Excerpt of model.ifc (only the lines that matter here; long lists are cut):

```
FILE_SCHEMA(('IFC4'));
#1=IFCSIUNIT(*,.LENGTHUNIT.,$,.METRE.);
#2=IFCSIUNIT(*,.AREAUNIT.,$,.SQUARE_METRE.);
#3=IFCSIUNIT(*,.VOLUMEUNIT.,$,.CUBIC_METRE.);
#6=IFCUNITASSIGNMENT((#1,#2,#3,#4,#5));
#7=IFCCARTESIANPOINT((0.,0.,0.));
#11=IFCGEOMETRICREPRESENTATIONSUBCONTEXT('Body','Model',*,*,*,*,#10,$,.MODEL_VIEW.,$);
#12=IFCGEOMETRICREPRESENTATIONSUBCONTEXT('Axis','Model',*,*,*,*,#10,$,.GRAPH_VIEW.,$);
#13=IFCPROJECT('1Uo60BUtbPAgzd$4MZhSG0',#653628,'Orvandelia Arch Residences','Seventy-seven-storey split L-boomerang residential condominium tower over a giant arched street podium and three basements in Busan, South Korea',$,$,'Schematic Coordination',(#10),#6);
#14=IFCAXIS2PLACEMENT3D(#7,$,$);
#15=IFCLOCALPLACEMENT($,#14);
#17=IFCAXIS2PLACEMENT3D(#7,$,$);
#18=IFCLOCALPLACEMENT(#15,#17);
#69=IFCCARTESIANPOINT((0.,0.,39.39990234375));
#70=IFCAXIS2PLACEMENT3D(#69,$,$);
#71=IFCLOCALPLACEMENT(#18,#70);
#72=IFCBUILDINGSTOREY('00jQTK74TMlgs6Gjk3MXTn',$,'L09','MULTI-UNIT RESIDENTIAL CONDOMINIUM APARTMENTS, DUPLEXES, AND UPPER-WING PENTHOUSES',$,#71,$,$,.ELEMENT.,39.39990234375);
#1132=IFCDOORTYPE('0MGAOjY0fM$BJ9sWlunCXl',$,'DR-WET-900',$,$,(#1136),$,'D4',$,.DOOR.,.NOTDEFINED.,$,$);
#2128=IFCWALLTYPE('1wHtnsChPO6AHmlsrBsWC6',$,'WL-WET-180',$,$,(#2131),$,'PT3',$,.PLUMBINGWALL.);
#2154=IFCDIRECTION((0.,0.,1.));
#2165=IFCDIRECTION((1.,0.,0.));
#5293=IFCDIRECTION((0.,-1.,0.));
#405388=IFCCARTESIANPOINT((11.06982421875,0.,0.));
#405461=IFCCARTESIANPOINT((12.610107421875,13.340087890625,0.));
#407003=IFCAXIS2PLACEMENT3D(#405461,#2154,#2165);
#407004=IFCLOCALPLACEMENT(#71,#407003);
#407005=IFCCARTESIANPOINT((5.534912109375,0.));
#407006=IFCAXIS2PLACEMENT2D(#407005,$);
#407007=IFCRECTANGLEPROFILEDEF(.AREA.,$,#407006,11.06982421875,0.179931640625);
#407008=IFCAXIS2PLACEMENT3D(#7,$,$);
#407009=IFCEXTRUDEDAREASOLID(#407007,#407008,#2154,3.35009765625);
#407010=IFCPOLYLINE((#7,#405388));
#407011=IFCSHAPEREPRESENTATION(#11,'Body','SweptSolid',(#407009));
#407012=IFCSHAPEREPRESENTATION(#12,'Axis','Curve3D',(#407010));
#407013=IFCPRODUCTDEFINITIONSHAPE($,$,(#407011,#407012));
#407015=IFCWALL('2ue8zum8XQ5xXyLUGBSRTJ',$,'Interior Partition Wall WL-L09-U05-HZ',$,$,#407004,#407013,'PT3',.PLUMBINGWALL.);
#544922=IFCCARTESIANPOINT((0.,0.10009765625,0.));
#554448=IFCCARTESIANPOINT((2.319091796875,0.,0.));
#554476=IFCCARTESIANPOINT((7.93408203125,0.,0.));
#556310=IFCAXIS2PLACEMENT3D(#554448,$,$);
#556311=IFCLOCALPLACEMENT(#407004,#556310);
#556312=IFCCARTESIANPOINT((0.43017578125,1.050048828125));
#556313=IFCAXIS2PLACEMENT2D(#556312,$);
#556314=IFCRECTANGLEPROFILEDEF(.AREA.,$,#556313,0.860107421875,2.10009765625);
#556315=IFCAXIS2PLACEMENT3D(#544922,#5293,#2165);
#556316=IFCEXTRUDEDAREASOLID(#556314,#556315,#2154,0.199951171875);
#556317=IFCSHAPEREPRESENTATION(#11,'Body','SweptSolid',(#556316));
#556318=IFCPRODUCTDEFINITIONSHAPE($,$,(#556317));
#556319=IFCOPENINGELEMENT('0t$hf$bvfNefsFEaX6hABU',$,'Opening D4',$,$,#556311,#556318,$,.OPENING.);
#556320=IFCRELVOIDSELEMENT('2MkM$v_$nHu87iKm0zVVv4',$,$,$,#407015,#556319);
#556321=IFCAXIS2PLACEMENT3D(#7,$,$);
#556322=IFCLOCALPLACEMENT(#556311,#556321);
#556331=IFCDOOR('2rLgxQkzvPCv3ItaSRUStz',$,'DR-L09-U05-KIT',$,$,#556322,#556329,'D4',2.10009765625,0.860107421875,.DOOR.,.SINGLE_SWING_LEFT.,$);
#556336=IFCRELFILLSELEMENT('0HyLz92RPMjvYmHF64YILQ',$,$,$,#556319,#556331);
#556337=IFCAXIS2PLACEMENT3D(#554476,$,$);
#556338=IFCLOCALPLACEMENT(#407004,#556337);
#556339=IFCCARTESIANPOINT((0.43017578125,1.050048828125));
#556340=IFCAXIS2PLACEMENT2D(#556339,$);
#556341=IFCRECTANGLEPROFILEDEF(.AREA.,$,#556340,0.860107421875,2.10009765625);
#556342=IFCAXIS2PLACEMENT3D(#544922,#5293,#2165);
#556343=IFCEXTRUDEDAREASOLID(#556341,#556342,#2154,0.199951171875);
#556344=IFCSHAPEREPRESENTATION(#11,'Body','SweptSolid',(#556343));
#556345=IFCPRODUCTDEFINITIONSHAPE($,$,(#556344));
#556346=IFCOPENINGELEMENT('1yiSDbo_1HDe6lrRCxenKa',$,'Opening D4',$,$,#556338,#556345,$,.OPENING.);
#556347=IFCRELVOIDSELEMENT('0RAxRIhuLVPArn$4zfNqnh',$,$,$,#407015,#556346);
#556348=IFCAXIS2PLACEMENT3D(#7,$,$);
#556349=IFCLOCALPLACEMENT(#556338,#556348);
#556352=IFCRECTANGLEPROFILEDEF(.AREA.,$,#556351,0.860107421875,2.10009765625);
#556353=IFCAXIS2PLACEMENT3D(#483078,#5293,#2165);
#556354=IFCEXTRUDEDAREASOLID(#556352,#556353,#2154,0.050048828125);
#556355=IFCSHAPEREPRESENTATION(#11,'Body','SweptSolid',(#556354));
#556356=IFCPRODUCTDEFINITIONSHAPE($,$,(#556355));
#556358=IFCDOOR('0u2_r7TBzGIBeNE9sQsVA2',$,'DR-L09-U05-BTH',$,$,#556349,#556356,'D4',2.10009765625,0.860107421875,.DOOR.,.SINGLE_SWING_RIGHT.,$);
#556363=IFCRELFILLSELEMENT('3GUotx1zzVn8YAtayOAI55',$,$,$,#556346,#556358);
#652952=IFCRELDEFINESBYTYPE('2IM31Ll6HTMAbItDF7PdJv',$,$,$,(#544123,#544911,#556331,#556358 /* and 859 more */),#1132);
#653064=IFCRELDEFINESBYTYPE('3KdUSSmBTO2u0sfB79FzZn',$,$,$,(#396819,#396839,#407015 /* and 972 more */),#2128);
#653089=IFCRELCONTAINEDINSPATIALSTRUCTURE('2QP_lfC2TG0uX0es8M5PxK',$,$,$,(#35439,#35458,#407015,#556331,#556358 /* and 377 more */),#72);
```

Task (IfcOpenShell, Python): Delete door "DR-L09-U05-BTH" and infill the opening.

```python
import ifcopenshell
import ifcopenshell.api.feature
import ifcopenshell.api.root
import ifcopenshell.geom
import ifcopenshell.util.shape

model = ifcopenshell.open("model.ifc")
settings = ifcopenshell.geom.settings()


def volume(element):
    """Net volume in cubic metres, openings subtracted."""
    shape = ifcopenshell.geom.create_shape(settings, element)
    return ifcopenshell.util.shape.get_volume(shape.geometry)


door = model.by_guid("0u2_r7TBzGIBeNE9sQsVA2")
opening = door.FillsVoids[0].RelatingOpeningElement
wall = opening.VoidsElements[0].RelatingBuildingElement
before = volume(wall)

ifcopenshell.api.root.remove_product(model, product=door)
ifcopenshell.api.feature.remove_feature(model, feature=opening)

after = volume(wall)

print(f"wall volume {before:.3f} -> {after:.3f} m3")

model.write("model_v2.ifc")
```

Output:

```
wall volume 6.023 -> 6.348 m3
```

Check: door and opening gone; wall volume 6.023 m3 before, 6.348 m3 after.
